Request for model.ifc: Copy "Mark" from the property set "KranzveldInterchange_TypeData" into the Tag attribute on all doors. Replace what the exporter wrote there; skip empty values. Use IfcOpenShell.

First a look at what the model holds.

```python
import ifcopenshell
import ifcopenshell.util.element

model = ifcopenshell.open("model.ifc")
print(model.schema)
doors = model.by_type("IfcDoor")
print(len(doors), "doors")
for e in doors[:8]:
    source = ifcopenshell.util.element.get_pset(e, "KranzveldInterchange_TypeData", "Mark")
    target = e.Tag
    print(e.id(), repr(source), repr(target), sep=" | ")
```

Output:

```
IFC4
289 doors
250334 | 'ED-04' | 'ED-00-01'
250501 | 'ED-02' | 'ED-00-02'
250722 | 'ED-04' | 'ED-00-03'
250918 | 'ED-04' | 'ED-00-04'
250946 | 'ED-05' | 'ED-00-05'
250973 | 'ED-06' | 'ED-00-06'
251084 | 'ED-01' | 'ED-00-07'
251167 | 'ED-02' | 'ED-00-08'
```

```python
import ifcopenshell
import ifcopenshell.util.element

model = ifcopenshell.open("model.ifc")

count = 0
for e in model.by_type("IfcDoor"):
    value = ifcopenshell.util.element.get_pset(e, "KranzveldInterchange_TypeData", "Mark")
    current = e.Tag
    if not value or not value.strip() or current == value:
        continue
    e.Tag = value
    count += 1

print(count, "doors updated")

model.write("model_updated.ifc")
```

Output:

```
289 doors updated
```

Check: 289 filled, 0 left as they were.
